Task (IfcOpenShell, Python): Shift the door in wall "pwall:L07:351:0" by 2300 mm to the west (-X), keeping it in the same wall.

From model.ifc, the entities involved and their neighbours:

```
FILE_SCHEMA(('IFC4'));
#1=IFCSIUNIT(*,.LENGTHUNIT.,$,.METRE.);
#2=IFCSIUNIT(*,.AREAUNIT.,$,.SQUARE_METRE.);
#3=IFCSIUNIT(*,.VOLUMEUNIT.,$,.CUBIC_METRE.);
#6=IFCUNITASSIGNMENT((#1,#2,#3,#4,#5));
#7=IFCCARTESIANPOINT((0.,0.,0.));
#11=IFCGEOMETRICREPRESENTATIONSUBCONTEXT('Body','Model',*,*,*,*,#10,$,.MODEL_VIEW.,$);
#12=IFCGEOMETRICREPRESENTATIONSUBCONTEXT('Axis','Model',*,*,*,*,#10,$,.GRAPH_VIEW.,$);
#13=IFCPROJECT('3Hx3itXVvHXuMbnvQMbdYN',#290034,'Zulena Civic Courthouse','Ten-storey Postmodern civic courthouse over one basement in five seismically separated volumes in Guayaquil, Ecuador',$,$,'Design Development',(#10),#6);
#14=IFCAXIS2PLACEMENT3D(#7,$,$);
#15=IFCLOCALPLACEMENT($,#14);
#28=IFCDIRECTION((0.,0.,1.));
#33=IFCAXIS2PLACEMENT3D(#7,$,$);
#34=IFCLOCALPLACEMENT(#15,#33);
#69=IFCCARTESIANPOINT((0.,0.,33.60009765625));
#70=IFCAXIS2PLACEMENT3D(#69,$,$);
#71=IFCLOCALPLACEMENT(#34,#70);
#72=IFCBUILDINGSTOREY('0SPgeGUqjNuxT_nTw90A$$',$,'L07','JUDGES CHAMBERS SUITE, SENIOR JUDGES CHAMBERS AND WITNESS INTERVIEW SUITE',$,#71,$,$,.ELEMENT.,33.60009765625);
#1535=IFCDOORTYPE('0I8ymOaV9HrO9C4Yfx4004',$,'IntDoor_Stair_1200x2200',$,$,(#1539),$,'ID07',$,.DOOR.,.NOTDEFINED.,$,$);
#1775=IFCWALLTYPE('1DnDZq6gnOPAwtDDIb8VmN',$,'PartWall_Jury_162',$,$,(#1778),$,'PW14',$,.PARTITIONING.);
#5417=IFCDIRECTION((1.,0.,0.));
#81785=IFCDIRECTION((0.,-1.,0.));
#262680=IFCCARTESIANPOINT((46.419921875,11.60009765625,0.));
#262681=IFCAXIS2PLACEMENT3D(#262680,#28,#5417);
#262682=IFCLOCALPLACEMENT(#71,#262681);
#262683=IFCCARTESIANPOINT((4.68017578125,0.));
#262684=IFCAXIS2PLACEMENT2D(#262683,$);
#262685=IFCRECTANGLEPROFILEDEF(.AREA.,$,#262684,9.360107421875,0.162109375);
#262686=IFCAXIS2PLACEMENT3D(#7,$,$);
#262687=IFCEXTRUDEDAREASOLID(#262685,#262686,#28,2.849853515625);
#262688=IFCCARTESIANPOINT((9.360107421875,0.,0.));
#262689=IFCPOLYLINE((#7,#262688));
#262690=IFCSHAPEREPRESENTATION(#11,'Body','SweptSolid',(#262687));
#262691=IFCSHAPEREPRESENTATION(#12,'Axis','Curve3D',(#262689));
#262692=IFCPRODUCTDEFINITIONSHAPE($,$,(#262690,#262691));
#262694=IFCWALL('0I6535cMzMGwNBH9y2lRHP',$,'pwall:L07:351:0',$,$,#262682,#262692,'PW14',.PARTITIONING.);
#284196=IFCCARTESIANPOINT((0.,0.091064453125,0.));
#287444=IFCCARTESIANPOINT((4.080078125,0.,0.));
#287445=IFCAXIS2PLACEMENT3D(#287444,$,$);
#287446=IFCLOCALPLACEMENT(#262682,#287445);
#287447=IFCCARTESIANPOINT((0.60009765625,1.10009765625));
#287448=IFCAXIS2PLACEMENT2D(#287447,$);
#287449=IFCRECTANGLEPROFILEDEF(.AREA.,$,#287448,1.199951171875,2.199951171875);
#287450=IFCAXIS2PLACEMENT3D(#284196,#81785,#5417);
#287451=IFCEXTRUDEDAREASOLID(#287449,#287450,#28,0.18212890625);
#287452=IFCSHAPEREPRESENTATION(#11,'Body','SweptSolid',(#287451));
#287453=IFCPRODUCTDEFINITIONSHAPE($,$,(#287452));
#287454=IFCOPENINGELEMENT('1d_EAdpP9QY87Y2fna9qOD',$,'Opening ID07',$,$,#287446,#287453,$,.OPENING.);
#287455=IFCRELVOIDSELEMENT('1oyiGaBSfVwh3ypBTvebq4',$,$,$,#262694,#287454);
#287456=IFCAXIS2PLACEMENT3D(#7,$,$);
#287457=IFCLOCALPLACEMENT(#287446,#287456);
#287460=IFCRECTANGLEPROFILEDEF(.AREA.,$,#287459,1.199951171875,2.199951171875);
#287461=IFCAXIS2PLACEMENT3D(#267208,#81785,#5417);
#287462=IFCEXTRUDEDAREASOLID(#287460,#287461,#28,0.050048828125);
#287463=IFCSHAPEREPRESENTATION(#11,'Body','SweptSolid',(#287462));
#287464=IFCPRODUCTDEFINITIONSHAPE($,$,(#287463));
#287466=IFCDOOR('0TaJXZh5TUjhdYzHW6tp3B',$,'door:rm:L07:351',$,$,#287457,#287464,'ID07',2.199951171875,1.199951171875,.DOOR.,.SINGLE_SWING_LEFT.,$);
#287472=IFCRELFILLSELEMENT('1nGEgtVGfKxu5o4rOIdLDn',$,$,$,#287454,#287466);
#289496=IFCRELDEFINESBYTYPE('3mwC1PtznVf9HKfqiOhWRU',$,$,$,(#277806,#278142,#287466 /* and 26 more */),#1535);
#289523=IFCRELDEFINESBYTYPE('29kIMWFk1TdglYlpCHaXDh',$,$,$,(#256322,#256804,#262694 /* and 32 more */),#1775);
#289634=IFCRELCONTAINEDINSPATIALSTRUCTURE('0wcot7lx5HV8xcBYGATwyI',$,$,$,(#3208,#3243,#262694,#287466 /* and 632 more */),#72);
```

```python
import ifcopenshell
import ifcopenshell.api.geometry
import ifcopenshell.util.placement

model = ifcopenshell.open("model.ifc")

door = model.by_id(287466)
opening = door.FillsVoids[0].RelatingOpeningElement
wall = opening.VoidsElements[0].RelatingBuildingElement

wall_matrix = ifcopenshell.util.placement.get_local_placement(wall.ObjectPlacement)
shift = wall_matrix[:3, 0] * -2.3
before = ifcopenshell.util.placement.get_local_placement(door.ObjectPlacement)[:3, 3].copy()

# The door is placed relative to its opening, so it follows when the opening moves.
matrix = ifcopenshell.util.placement.get_local_placement(opening.ObjectPlacement)
matrix[:3, 3] += shift
ifcopenshell.api.geometry.edit_object_placement(
    model, product=opening, matrix=matrix, is_si=False, should_transform_children=True
)

after = ifcopenshell.util.placement.get_local_placement(door.ObjectPlacement)[:3, 3]
print("door moved by", (after - before).round(3) + 0.0)

model.write("model_rev.ifc")
```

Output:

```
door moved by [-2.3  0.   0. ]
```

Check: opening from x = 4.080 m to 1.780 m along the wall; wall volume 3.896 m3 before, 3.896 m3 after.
